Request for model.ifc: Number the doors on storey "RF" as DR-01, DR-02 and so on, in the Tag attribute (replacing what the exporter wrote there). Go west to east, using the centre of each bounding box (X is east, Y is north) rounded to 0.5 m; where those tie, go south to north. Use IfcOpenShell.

First a look at what the model holds.

```python
import ifcopenshell
import ifcopenshell.util.element
import ifcopenshell.util.placement

model = ifcopenshell.open("model.ifc")
print(model.schema)
storey = next(s for s in model.by_type("IfcBuildingStorey") if s.Name == "RF")
doors = [e for e in ifcopenshell.util.element.get_decomposition(storey) if e.is_a("IfcDoor")]
for e in sorted(doors, key=lambda e: e.id()):
    origin = ifcopenshell.util.placement.get_local_placement(e.ObjectPlacement)[:3, 3]
    print(e.id(), e.Tag, e.Name, origin.round(2) + 0.0, sep=" | ")
```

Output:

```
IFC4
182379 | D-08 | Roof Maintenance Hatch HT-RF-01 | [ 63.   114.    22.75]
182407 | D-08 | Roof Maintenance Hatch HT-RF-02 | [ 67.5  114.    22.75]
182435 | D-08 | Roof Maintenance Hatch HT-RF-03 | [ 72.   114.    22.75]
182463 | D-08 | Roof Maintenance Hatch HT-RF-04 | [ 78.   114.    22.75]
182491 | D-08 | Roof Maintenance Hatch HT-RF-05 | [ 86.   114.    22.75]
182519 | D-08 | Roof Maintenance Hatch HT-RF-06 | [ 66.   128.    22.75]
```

```python
import ifcopenshell
import ifcopenshell.geom
import ifcopenshell.util.element
import ifcopenshell.util.shape

model = ifcopenshell.open("model.ifc")
settings = ifcopenshell.geom.settings()
settings.set("use-world-coords", True)


def centre(element):
    shape = ifcopenshell.geom.create_shape(settings, element)
    return ifcopenshell.util.shape.get_bbox_centroid(shape.geometry)


storey = next(s for s in model.by_type("IfcBuildingStorey") if s.Name == "RF")
doors = [e for e in ifcopenshell.util.element.get_decomposition(storey) if e.is_a("IfcDoor")]

# Insertion points can sit at a corner or the storey origin, so sort by the geometry (in metres).
centres = {e: centre(e) for e in doors}
doors.sort(key=lambda e: (round(centres[e][0] / 0.5), centres[e][1]))

for i, e in enumerate(doors, start=1):
    number = f"DR-{i:02d}"
    e.Tag = number
    print(e.id(), number)

model.write("model_updated.ifc")
```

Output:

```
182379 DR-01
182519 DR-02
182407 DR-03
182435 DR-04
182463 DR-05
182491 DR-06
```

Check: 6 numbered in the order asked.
